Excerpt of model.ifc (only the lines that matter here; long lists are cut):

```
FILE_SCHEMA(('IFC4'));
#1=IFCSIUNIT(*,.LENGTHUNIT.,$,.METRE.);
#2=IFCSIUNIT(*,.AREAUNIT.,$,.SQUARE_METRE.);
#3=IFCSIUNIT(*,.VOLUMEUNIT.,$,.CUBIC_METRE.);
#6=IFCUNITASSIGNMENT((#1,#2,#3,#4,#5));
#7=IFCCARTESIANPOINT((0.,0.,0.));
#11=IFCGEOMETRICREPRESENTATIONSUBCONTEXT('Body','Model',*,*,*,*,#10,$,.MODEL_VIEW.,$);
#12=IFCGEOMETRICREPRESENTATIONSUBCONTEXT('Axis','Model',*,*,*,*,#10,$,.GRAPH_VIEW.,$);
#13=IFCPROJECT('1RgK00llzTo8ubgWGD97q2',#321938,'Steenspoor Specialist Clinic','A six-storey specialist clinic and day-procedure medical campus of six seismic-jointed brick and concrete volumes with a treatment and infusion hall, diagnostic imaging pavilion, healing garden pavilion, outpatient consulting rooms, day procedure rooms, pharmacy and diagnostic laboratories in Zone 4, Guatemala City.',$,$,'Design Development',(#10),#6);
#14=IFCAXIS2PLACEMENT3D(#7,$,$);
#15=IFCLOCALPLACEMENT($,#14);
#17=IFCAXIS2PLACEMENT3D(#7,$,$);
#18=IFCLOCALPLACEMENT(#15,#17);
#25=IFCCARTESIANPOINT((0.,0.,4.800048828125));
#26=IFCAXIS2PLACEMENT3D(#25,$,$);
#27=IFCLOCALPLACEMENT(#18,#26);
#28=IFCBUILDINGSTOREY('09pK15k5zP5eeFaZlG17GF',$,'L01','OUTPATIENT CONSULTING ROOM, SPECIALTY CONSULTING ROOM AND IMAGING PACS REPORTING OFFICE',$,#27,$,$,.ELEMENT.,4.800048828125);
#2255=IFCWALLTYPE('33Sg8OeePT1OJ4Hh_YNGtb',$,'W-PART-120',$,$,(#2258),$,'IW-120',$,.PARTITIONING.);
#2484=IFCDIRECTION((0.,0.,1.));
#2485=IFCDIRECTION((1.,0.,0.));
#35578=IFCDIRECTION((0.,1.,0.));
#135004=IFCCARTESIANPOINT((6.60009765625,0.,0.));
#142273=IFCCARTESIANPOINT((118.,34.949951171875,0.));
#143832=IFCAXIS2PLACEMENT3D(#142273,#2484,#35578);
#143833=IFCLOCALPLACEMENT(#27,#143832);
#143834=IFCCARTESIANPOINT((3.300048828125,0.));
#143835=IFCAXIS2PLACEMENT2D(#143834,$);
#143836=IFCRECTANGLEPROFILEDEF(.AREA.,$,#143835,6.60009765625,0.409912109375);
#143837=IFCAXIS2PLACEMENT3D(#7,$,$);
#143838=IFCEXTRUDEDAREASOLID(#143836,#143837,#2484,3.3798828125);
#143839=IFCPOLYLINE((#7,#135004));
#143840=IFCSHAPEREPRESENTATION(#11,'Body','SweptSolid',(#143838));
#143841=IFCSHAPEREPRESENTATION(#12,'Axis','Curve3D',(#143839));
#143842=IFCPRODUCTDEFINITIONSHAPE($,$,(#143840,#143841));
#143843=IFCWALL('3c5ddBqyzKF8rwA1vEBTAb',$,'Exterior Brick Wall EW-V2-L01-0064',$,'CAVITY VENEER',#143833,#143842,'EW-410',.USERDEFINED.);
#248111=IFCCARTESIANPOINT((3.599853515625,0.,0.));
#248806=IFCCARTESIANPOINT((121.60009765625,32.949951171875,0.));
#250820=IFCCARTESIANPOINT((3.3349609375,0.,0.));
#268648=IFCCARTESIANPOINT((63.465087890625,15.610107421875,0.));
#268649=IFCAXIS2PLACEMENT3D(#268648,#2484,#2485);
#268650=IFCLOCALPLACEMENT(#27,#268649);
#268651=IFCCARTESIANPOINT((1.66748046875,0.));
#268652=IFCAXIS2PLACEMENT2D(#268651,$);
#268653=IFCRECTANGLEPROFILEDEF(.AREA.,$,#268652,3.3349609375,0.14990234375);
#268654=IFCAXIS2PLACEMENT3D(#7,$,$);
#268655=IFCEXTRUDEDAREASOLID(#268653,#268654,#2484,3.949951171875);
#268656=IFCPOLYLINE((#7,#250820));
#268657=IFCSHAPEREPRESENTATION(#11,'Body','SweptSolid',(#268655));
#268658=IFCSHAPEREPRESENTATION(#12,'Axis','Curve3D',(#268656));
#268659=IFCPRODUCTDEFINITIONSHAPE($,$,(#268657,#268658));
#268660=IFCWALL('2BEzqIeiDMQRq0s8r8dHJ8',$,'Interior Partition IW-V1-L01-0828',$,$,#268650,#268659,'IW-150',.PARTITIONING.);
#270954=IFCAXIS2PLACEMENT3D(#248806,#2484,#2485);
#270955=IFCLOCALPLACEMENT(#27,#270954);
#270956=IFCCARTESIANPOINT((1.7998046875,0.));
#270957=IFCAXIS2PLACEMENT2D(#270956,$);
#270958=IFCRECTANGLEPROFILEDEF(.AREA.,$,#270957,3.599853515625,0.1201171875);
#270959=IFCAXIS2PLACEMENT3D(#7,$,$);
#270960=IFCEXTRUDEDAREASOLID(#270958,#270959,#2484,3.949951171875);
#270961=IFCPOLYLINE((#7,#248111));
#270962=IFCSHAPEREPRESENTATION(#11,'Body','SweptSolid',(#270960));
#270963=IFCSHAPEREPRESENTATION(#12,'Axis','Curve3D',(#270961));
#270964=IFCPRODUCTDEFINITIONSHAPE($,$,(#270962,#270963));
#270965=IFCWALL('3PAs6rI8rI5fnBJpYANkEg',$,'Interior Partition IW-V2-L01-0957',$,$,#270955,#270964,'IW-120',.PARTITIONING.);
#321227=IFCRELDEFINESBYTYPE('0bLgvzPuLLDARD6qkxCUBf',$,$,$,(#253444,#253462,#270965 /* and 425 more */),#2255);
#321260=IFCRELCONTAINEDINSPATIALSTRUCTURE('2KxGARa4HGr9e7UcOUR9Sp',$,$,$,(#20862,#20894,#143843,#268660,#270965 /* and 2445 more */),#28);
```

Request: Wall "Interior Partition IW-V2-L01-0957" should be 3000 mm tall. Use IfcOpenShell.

```python
import ifcopenshell
import ifcopenshell.geom
import ifcopenshell.util.representation
import ifcopenshell.util.shape
import ifcopenshell.util.unit

model = ifcopenshell.open("model.ifc")
unit_scale = ifcopenshell.util.unit.calculate_unit_scale(model)
settings = ifcopenshell.geom.settings()


def volume(element):
    """Net volume in cubic metres, openings subtracted."""
    shape = ifcopenshell.geom.create_shape(settings, element)
    return ifcopenshell.util.shape.get_volume(shape.geometry)


wall = model.by_guid("3PAs6rI8rI5fnBJpYANkEg")
before = volume(wall)

body = ifcopenshell.util.representation.get_representation(wall, "Model", "Body")
solid = body.Items[0]
old_height = solid.Depth
solid.Depth = 3 / unit_scale
after = volume(wall)

print(f"height {old_height:g} -> {solid.Depth:g}, volume {before:.3f} -> {after:.3f} m3")

model.write("model_v2.ifc")
```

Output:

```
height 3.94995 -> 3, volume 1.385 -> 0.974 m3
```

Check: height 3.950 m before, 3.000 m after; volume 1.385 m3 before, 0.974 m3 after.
